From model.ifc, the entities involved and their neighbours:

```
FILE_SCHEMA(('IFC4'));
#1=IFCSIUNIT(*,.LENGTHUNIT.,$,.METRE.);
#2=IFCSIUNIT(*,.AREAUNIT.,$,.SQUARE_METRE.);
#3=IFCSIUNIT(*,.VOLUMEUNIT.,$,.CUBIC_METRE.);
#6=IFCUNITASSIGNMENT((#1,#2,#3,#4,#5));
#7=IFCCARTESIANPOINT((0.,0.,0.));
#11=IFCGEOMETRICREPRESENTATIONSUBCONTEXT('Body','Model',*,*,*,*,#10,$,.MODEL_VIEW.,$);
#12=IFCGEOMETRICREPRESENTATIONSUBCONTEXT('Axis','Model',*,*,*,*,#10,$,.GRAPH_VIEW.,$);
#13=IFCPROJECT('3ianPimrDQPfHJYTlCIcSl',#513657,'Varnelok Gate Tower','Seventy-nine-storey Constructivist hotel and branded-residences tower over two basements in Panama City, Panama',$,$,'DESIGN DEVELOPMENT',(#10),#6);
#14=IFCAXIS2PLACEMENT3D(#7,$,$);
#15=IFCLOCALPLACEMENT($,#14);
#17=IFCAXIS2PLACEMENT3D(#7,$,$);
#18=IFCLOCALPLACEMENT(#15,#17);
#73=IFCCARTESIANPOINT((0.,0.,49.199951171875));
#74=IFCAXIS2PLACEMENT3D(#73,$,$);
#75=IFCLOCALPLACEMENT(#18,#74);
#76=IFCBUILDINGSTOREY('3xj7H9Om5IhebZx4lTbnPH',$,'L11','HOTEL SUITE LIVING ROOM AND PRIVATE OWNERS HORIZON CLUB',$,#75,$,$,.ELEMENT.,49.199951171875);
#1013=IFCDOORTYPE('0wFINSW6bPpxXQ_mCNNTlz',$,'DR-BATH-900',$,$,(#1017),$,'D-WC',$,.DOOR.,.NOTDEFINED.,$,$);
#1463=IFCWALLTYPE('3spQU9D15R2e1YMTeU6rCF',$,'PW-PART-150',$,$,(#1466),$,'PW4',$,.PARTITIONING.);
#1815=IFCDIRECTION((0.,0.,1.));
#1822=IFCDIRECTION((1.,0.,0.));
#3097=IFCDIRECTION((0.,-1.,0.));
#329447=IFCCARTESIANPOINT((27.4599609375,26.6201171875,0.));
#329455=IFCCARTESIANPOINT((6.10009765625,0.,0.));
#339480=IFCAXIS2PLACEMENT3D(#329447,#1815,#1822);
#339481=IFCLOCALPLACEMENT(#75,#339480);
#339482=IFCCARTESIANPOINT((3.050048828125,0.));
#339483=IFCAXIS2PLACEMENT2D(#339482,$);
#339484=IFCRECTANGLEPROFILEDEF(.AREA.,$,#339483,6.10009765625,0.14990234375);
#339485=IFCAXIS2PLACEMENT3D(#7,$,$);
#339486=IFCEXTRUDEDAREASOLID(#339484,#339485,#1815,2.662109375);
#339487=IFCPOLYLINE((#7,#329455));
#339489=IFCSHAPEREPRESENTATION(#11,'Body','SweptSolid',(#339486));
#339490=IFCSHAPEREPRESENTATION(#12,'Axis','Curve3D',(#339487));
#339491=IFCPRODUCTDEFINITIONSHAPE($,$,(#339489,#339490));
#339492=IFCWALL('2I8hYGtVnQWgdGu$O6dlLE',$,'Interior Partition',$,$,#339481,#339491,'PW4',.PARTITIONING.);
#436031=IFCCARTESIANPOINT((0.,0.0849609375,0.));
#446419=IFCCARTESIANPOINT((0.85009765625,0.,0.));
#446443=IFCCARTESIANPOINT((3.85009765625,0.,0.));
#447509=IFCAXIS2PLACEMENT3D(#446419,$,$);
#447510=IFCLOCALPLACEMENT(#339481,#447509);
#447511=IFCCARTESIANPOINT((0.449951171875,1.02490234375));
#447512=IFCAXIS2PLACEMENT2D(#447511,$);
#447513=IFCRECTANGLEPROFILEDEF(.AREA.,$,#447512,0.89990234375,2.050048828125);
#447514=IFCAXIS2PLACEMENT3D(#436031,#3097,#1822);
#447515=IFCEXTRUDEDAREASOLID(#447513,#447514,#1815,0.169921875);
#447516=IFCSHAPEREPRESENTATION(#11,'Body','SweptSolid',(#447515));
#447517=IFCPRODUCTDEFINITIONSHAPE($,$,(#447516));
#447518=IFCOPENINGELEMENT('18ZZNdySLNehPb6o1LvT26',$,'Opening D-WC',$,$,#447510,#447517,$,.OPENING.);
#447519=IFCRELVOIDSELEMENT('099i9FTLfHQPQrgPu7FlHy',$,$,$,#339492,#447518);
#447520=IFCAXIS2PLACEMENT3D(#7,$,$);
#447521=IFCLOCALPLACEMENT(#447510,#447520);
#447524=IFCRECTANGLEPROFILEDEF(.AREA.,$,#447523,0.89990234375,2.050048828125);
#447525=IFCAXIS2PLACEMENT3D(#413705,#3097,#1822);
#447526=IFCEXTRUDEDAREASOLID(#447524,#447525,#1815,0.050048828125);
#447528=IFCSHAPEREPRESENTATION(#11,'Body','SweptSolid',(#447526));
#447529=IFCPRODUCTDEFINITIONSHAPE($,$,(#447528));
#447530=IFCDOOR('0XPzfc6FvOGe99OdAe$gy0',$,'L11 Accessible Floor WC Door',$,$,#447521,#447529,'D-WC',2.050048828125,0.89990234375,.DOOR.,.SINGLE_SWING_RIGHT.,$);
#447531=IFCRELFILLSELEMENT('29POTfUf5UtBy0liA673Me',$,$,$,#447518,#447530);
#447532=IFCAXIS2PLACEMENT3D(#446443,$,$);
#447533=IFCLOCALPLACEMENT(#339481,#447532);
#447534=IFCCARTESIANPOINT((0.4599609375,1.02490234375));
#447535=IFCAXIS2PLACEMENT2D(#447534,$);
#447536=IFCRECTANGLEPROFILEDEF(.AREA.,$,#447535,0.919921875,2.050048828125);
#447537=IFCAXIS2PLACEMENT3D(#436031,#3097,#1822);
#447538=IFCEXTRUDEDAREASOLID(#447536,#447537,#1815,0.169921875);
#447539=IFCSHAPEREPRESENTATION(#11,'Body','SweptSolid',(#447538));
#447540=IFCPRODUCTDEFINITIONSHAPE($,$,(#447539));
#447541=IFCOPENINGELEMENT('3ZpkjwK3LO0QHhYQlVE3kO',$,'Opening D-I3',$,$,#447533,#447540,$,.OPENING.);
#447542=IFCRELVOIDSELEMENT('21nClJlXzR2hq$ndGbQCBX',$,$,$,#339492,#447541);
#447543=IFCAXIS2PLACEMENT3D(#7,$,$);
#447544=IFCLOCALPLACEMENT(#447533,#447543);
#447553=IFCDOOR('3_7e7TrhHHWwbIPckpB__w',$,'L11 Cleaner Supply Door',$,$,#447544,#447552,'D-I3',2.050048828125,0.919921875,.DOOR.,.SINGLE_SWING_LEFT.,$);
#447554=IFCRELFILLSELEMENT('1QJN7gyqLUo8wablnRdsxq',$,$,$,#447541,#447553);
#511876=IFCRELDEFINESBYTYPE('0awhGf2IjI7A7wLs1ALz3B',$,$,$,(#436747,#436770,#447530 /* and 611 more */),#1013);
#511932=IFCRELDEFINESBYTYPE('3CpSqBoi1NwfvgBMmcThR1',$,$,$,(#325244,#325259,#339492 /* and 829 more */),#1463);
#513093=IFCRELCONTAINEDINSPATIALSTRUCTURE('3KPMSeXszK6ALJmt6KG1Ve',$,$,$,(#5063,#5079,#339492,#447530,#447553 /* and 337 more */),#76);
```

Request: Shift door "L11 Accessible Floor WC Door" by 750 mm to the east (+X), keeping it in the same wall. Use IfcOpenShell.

```python
import ifcopenshell
import ifcopenshell.api.geometry
import ifcopenshell.util.placement

model = ifcopenshell.open("model.ifc")

door = model.by_guid("0XPzfc6FvOGe99OdAe$gy0")
opening = door.FillsVoids[0].RelatingOpeningElement
wall = opening.VoidsElements[0].RelatingBuildingElement

wall_matrix = ifcopenshell.util.placement.get_local_placement(wall.ObjectPlacement)
shift = wall_matrix[:3, 0] * 0.75
before = ifcopenshell.util.placement.get_local_placement(door.ObjectPlacement)[:3, 3].copy()

# The door is placed relative to its opening, so it follows when the opening moves.
matrix = ifcopenshell.util.placement.get_local_placement(opening.ObjectPlacement)
matrix[:3, 3] += shift
ifcopenshell.api.geometry.edit_object_placement(
    model, product=opening, matrix=matrix, is_si=False, should_transform_children=True
)

after = ifcopenshell.util.placement.get_local_placement(door.ObjectPlacement)[:3, 3]
print("door moved by", (after - before).round(3) + 0.0)

model.write("model-out.ifc")
```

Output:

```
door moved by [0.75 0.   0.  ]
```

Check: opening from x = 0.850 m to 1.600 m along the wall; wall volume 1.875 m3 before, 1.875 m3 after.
